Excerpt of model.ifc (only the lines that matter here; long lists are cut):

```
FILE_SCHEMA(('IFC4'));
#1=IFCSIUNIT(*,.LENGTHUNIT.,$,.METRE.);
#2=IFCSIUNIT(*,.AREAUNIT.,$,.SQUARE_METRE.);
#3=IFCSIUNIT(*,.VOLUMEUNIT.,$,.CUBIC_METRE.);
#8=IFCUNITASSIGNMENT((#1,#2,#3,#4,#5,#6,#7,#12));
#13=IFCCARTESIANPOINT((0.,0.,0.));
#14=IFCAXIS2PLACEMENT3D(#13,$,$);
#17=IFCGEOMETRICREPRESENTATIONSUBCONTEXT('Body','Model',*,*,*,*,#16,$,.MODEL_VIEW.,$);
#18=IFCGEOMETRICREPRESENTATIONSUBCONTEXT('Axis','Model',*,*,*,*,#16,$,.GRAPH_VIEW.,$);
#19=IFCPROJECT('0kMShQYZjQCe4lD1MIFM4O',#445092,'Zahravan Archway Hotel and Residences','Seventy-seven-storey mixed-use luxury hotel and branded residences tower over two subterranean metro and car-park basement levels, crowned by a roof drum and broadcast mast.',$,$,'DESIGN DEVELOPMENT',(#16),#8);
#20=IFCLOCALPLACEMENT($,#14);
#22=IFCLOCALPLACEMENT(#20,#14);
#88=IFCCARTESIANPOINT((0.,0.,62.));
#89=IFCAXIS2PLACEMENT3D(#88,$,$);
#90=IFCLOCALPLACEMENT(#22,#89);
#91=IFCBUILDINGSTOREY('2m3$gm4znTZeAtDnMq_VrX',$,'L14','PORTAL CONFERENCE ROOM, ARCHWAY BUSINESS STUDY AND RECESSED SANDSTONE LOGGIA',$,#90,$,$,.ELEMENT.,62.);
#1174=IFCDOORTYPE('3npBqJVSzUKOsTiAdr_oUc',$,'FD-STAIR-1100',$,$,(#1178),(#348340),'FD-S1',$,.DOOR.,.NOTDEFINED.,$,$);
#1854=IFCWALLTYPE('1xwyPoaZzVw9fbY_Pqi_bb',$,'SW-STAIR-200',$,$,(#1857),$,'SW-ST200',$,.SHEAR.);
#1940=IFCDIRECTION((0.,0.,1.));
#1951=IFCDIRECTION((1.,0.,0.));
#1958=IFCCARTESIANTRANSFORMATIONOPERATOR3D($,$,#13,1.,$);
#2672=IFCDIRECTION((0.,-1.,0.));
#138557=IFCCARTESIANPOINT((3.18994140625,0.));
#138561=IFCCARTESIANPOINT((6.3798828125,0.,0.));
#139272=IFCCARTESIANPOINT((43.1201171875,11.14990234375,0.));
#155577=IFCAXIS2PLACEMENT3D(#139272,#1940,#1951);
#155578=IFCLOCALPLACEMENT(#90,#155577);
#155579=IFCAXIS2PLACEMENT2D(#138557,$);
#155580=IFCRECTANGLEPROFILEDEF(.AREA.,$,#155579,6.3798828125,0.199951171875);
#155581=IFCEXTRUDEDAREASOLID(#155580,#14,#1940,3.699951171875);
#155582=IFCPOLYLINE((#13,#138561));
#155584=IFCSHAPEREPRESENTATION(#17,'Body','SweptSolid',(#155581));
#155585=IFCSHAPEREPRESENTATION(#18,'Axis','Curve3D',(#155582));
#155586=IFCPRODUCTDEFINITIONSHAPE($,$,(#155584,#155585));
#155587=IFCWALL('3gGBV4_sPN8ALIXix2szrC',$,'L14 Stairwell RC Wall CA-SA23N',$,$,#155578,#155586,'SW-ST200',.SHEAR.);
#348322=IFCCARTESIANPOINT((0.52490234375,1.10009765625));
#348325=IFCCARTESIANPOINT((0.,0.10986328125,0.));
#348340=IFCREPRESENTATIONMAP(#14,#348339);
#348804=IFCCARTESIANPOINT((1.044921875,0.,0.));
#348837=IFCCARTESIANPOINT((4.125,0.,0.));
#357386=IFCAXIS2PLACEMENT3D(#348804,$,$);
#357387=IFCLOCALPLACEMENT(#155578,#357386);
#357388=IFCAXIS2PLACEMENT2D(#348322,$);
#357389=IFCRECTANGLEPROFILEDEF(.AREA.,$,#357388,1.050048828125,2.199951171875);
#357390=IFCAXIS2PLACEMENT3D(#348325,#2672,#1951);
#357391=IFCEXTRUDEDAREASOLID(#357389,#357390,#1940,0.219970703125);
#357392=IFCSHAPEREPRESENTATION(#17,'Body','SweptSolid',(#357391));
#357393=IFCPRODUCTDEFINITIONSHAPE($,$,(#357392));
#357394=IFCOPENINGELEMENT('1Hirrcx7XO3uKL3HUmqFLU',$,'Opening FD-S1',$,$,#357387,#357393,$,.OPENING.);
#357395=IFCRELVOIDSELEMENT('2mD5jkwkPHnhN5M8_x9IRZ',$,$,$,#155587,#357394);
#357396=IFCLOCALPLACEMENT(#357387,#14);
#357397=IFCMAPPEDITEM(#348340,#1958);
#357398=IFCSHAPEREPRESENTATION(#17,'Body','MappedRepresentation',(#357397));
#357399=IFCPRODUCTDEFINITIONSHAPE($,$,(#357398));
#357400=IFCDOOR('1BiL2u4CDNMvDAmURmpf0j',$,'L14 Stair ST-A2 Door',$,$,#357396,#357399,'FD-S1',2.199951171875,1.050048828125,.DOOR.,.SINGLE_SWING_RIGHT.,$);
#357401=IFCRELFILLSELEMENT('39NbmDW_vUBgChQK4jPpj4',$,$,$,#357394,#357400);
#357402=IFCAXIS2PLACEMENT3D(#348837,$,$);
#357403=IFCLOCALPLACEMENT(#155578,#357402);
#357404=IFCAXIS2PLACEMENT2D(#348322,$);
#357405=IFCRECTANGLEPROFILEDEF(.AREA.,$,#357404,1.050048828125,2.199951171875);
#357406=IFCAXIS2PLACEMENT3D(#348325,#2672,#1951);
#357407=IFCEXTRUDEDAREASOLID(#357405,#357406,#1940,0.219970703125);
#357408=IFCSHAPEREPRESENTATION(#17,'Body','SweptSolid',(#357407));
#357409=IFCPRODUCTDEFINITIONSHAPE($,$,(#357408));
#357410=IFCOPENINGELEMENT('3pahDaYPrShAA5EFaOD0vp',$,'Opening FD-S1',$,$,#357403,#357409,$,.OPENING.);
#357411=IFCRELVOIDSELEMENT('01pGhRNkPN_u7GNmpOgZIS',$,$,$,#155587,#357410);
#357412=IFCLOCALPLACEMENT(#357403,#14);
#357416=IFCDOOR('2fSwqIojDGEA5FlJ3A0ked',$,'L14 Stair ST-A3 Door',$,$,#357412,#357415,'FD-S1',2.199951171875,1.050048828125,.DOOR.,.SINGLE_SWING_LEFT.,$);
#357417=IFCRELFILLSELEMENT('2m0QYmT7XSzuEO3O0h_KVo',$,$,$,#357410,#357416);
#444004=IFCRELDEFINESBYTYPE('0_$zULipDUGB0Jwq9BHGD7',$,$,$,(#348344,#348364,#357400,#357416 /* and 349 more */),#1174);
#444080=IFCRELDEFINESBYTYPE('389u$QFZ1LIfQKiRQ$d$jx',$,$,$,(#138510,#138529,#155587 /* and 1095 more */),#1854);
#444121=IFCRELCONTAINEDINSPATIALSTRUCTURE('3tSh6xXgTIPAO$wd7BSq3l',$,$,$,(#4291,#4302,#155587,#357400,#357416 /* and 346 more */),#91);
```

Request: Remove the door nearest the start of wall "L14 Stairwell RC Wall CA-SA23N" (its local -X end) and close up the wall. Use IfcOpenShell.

```python
import ifcopenshell
import ifcopenshell.api.feature
import ifcopenshell.api.root
import ifcopenshell.geom
import ifcopenshell.util.shape

model = ifcopenshell.open("model.ifc")
settings = ifcopenshell.geom.settings()


def volume(element):
    """Net volume in cubic metres, openings subtracted."""
    shape = ifcopenshell.geom.create_shape(settings, element)
    return ifcopenshell.util.shape.get_volume(shape.geometry)


door = model.by_guid("1BiL2u4CDNMvDAmURmpf0j")
opening = door.FillsVoids[0].RelatingOpeningElement
wall = opening.VoidsElements[0].RelatingBuildingElement
before = volume(wall)

ifcopenshell.api.root.remove_product(model, product=door)
ifcopenshell.api.feature.remove_feature(model, feature=opening)

after = volume(wall)

print(f"wall volume {before:.3f} -> {after:.3f} m3")

model.write("model-out.ifc")
```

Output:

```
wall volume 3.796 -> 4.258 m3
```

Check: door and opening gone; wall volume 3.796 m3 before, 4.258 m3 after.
